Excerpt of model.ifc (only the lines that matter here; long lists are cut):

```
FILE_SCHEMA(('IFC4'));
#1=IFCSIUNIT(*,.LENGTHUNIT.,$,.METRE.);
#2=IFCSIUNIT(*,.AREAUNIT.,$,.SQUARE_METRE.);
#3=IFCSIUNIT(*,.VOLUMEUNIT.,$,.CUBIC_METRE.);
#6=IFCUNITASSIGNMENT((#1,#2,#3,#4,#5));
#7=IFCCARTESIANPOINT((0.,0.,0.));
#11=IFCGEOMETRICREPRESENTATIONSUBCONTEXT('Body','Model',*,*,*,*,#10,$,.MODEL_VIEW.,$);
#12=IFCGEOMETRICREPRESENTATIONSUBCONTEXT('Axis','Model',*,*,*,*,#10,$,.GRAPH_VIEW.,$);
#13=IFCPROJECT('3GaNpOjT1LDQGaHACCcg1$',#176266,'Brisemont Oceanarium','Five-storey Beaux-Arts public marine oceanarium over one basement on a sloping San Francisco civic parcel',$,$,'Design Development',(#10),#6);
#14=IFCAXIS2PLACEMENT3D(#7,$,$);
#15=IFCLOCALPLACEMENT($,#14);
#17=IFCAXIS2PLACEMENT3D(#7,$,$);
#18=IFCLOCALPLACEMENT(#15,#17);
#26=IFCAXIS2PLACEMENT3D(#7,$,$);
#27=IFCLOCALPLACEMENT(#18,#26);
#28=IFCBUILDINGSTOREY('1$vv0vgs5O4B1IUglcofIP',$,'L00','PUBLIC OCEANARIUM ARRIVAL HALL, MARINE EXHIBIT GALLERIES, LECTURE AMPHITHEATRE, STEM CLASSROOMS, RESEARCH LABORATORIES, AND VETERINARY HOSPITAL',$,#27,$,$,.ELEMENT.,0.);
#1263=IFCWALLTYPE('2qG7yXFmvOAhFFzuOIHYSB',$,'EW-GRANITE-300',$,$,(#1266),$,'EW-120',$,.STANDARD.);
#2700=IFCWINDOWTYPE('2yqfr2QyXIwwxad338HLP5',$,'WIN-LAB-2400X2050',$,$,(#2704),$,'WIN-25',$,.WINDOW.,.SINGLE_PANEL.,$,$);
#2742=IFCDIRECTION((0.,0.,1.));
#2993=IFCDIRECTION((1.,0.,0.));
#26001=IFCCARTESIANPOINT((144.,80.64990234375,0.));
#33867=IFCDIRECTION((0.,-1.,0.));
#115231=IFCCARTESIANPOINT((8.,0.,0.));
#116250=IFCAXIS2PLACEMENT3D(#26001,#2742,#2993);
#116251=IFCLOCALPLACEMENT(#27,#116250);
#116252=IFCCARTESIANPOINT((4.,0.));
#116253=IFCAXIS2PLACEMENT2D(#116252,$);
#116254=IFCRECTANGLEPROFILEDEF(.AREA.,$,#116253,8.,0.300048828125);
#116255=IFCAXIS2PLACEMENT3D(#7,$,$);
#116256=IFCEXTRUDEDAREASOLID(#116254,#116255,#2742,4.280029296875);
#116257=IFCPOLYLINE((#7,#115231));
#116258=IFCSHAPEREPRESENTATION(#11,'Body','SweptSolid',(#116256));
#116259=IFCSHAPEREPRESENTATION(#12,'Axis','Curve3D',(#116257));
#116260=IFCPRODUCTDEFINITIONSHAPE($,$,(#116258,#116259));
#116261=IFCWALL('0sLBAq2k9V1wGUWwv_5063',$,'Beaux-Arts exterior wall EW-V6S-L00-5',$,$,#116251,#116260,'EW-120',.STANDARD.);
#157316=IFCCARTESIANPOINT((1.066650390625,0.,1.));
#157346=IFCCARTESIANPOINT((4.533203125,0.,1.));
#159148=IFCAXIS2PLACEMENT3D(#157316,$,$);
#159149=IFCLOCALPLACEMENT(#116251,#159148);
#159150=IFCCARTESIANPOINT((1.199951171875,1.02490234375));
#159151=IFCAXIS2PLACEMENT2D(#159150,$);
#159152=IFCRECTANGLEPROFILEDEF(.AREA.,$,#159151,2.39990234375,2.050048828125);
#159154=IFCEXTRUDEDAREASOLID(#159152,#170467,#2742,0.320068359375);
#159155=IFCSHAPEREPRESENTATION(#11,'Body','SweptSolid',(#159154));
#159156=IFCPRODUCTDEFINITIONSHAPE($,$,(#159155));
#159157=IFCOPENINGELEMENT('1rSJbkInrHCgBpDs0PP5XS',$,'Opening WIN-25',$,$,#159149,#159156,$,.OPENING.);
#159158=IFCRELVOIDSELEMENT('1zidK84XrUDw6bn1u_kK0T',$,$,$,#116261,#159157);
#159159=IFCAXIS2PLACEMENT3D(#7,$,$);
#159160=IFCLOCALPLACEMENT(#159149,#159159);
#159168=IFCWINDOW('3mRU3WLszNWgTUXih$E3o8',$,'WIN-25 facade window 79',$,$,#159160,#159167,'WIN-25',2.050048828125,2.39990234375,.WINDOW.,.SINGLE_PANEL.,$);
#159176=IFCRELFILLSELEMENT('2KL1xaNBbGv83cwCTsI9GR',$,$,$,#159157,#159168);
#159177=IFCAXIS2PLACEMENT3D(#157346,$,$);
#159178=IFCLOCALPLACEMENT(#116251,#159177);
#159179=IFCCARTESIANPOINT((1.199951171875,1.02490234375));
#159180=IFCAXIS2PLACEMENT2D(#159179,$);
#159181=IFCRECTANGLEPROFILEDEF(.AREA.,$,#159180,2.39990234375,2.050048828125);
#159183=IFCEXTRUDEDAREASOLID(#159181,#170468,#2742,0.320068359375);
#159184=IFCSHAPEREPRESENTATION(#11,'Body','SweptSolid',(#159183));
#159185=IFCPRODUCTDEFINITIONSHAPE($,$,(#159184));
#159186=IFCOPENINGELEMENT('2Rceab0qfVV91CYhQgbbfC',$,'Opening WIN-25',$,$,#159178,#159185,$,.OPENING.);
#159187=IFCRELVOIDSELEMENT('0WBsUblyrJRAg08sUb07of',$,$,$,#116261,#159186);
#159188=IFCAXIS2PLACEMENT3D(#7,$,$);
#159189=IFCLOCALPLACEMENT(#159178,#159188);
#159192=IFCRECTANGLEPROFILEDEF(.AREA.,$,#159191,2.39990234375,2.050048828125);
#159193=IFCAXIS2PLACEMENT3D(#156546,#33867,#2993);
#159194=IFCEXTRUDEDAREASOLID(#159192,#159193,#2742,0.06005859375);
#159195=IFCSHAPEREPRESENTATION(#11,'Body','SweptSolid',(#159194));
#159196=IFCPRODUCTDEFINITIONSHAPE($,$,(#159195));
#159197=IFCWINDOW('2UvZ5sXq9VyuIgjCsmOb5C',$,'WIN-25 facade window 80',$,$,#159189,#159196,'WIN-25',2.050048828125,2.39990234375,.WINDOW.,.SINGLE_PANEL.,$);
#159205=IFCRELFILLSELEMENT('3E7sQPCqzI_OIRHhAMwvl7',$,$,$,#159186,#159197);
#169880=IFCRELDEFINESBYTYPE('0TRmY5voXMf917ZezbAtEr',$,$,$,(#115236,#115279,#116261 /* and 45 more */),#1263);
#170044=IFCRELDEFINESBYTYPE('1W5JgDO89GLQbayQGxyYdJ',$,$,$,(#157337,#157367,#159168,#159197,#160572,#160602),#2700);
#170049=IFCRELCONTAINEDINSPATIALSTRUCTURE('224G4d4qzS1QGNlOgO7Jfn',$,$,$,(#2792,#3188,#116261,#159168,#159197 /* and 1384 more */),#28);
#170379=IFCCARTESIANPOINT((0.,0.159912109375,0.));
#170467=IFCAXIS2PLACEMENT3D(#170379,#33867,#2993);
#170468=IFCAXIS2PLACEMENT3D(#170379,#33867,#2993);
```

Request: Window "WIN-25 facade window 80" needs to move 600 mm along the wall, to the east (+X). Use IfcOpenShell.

```python
import ifcopenshell
import ifcopenshell.api.geometry
import ifcopenshell.util.placement
import ifcopenshell.util.unit

model = ifcopenshell.open("model.ifc")
unit_scale = ifcopenshell.util.unit.calculate_unit_scale(model)

window = model.by_guid("2UvZ5sXq9VyuIgjCsmOb5C")
opening = window.FillsVoids[0].RelatingOpeningElement
wall = opening.VoidsElements[0].RelatingBuildingElement

wall_matrix = ifcopenshell.util.placement.get_local_placement(wall.ObjectPlacement)
shift = wall_matrix[:3, 0] * 0.6 / unit_scale
before = ifcopenshell.util.placement.get_local_placement(window.ObjectPlacement)[:3, 3].copy()

# The window is placed relative to its opening, so it follows when the opening moves.
matrix = ifcopenshell.util.placement.get_local_placement(opening.ObjectPlacement)
matrix[:3, 3] += shift
ifcopenshell.api.geometry.edit_object_placement(
    model, product=opening, matrix=matrix, is_si=False, should_transform_children=True
)

after = ifcopenshell.util.placement.get_local_placement(window.ObjectPlacement)[:3, 3]
print("window moved by", (after - before).round(3) + 0.0)

model.write("model-out.ifc")
```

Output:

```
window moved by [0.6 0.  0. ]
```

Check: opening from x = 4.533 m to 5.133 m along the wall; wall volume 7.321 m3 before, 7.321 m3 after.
